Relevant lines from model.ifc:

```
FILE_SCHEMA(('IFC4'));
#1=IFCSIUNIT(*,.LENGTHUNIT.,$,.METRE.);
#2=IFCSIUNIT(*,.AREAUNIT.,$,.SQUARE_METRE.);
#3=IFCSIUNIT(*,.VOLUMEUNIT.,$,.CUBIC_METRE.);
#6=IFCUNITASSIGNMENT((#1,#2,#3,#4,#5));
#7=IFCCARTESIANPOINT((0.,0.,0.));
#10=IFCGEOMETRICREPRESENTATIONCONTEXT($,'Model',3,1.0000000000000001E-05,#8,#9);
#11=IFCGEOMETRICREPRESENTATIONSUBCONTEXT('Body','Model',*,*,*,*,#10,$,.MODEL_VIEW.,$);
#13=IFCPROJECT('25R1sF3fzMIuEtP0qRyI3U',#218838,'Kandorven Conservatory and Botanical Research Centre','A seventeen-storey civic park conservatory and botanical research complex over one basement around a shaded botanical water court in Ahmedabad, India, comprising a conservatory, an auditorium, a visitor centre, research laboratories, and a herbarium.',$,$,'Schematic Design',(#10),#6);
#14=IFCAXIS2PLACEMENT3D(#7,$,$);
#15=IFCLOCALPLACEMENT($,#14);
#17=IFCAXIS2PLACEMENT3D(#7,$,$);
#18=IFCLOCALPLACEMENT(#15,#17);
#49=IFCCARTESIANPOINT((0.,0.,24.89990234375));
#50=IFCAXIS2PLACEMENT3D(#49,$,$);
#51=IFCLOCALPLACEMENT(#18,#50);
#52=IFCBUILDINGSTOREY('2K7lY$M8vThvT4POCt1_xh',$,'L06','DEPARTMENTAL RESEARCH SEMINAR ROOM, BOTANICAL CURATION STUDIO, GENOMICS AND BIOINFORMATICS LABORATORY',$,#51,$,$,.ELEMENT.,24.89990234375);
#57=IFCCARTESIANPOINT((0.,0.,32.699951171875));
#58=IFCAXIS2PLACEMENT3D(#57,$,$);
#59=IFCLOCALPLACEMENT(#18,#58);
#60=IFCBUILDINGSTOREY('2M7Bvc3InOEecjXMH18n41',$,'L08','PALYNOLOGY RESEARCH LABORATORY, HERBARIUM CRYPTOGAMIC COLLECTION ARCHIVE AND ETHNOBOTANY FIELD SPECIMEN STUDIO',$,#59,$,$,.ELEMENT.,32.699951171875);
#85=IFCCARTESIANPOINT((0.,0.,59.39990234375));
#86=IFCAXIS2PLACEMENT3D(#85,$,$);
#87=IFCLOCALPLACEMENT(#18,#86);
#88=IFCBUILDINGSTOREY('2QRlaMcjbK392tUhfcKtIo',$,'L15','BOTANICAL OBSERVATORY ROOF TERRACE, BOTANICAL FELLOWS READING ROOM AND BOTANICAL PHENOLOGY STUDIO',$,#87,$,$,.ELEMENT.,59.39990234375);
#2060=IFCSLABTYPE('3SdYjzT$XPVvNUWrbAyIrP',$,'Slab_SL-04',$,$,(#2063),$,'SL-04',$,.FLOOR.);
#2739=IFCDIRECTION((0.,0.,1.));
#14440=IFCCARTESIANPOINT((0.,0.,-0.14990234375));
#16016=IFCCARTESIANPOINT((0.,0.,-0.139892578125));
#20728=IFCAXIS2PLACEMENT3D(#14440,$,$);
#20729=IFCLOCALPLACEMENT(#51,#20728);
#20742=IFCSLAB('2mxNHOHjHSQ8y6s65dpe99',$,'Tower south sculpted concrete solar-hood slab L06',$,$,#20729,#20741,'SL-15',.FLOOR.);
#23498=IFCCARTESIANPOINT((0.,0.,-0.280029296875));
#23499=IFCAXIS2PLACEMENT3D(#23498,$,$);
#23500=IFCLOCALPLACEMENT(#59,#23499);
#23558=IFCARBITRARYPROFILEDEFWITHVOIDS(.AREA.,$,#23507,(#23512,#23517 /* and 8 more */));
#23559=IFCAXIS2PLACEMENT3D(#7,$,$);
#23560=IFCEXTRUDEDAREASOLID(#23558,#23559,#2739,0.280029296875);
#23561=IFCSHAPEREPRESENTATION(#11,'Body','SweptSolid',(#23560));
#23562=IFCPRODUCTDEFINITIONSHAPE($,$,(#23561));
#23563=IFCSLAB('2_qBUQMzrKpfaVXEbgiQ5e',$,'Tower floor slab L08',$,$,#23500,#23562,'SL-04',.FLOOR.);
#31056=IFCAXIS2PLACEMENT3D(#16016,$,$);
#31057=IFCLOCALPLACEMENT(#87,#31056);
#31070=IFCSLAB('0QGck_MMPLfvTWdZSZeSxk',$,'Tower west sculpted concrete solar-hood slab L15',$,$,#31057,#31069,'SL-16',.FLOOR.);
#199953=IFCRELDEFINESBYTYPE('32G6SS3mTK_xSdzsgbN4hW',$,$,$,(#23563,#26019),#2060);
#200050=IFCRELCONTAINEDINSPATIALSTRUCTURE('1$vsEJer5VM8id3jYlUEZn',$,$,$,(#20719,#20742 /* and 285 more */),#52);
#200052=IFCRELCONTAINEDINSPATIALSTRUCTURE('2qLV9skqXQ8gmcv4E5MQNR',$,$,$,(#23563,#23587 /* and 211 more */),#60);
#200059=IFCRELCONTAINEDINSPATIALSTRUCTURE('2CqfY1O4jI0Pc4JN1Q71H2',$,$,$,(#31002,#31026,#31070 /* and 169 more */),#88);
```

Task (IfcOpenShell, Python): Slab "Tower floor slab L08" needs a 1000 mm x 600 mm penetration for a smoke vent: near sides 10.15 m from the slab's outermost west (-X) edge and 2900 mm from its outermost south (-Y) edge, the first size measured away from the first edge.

```python
import numpy as np
import ifcopenshell
import ifcopenshell.api.feature
import ifcopenshell.api.geometry
import ifcopenshell.api.root
import ifcopenshell.geom
import ifcopenshell.util.placement
import ifcopenshell.util.representation
import ifcopenshell.util.shape
import ifcopenshell.util.unit

model = ifcopenshell.open("model.ifc")
unit_scale = ifcopenshell.util.unit.calculate_unit_scale(model)
settings = ifcopenshell.geom.settings()


def volume(element):
    """Net volume in cubic metres, openings subtracted."""
    shape = ifcopenshell.geom.create_shape(settings, element)
    return ifcopenshell.util.shape.get_volume(shape.geometry)


slab = model.by_guid("2_qBUQMzrKpfaVXEbgiQ5e")
before = volume(slab)

# Extent in the slab's own axes, in metres. The edges named are its -X and -Y sides.
slab_shape = ifcopenshell.geom.create_shape(settings, slab)
vertices = ifcopenshell.util.shape.get_vertices(slab_shape.geometry)
x_min, y_min, bottom = vertices.min(axis=0)
top = vertices[:, 2].max()

opening = ifcopenshell.api.root.create_entity(model, ifc_class="IfcOpeningElement", name="Smoke vent opening", predefined_type="OPENING")
context = ifcopenshell.util.representation.get_context(model, "Model", "Body", "MODEL_VIEW")
width, depth = 1, 0.6
outline = [(0.0, 0.0), (width, 0.0), (width, depth), (0.0, depth), (0.0, 0.0)]
# Overshoot both faces by 50 mm so the cut is clean.
shape = ifcopenshell.api.geometry.add_slab_representation(
    model, context=context, depth=top - bottom + 0.1, polyline=outline
)
ifcopenshell.api.geometry.assign_representation(model, product=opening, representation=shape)

matrix = ifcopenshell.util.placement.get_local_placement(slab.ObjectPlacement)
matrix[:, 3] = matrix @ np.append(np.array([x_min + 10.15, y_min + 2.9, bottom - 0.05]) / unit_scale, 1.0)
ifcopenshell.api.geometry.edit_object_placement(model, product=opening, matrix=matrix, is_si=False)
ifcopenshell.api.feature.add_feature(model, feature=opening, element=slab)

after = volume(slab)

print(f"slab volume {before:.3f} -> {after:.3f} m3")

model.write("model_edited.ifc")
```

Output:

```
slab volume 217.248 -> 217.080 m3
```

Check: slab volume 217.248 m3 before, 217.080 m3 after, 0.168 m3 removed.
